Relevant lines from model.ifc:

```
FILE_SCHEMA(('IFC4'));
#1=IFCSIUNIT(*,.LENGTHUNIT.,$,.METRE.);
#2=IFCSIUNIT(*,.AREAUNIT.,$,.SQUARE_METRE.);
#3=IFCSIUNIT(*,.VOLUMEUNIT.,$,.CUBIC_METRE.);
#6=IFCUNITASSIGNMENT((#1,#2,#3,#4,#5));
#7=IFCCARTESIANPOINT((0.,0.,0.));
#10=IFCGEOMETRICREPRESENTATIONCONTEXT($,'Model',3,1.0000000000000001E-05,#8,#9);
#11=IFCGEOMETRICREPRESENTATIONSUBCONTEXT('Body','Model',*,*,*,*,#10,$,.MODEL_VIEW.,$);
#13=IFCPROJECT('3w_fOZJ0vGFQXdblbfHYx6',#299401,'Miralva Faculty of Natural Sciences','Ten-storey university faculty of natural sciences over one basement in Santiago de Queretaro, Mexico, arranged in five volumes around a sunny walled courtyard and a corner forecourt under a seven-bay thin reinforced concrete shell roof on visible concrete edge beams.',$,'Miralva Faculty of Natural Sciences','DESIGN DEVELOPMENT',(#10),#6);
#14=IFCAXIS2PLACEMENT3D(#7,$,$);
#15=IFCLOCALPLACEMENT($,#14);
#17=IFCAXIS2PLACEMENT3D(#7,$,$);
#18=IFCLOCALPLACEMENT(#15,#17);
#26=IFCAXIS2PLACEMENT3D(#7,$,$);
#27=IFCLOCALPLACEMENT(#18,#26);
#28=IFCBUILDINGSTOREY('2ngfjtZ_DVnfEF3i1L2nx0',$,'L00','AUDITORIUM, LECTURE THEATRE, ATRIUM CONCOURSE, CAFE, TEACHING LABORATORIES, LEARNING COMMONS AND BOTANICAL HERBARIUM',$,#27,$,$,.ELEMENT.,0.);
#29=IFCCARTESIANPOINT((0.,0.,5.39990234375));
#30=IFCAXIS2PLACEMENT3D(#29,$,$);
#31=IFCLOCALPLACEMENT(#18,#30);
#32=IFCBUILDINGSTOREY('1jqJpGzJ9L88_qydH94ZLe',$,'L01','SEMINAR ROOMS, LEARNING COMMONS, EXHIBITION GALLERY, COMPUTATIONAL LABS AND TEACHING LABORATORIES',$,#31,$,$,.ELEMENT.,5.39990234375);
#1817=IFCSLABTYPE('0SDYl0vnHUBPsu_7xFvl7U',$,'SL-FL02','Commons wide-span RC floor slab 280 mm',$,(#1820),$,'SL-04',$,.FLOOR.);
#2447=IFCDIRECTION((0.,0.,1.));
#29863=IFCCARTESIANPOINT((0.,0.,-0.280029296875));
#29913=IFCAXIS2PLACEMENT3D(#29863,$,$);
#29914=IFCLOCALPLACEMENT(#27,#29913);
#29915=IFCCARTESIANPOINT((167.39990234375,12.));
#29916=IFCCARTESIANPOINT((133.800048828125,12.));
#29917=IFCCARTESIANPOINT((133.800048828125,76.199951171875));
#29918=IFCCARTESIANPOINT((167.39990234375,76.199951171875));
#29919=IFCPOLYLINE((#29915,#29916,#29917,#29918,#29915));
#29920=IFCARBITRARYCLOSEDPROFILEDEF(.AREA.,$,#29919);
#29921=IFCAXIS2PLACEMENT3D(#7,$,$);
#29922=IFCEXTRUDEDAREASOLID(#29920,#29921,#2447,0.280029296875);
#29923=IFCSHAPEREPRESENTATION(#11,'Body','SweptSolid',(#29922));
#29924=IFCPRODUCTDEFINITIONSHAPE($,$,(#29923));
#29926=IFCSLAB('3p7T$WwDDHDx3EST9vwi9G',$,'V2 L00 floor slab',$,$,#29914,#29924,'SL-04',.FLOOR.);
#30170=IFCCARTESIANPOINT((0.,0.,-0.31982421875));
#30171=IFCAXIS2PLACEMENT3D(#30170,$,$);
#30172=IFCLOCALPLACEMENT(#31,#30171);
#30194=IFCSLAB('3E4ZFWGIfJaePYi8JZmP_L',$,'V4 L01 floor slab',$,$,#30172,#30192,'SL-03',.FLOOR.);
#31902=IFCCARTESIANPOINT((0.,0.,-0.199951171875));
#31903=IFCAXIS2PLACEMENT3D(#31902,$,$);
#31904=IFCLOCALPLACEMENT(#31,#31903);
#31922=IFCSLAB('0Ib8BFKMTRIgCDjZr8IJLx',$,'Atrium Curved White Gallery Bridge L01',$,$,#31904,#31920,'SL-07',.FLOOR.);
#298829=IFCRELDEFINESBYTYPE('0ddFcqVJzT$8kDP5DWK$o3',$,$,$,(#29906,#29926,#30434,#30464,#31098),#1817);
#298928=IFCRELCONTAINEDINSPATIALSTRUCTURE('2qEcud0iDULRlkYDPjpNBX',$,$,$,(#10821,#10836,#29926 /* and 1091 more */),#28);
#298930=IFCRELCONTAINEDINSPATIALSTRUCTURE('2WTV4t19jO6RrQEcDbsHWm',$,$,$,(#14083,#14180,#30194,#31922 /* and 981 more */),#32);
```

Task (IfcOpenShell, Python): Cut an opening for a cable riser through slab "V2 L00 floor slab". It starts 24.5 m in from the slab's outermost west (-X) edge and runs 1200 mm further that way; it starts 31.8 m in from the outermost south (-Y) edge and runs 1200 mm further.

```python
import numpy as np
import ifcopenshell
import ifcopenshell.api.feature
import ifcopenshell.api.geometry
import ifcopenshell.api.root
import ifcopenshell.geom
import ifcopenshell.util.placement
import ifcopenshell.util.representation
import ifcopenshell.util.shape
import ifcopenshell.util.unit

model = ifcopenshell.open("model.ifc")
unit_scale = ifcopenshell.util.unit.calculate_unit_scale(model)
settings = ifcopenshell.geom.settings()


def volume(element):
    """Net volume in cubic metres, openings subtracted."""
    shape = ifcopenshell.geom.create_shape(settings, element)
    return ifcopenshell.util.shape.get_volume(shape.geometry)


slab = model.by_guid("3p7T$WwDDHDx3EST9vwi9G")
before = volume(slab)

# Extent in the slab's own axes, in metres. The edges named are its -X and -Y sides.
slab_shape = ifcopenshell.geom.create_shape(settings, slab)
vertices = ifcopenshell.util.shape.get_vertices(slab_shape.geometry)
x_min, y_min, bottom = vertices.min(axis=0)
top = vertices[:, 2].max()

opening = ifcopenshell.api.root.create_entity(model, ifc_class="IfcOpeningElement", name="Cable riser opening", predefined_type="OPENING")
context = ifcopenshell.util.representation.get_context(model, "Model", "Body", "MODEL_VIEW")
width, depth = 1.2, 1.2
outline = [(0.0, 0.0), (width, 0.0), (width, depth), (0.0, depth), (0.0, 0.0)]
# Overshoot both faces by 50 mm so the cut is clean.
shape = ifcopenshell.api.geometry.add_slab_representation(
    model, context=context, depth=top - bottom + 0.1, polyline=outline
)
ifcopenshell.api.geometry.assign_representation(model, product=opening, representation=shape)

matrix = ifcopenshell.util.placement.get_local_placement(slab.ObjectPlacement)
matrix[:, 3] = matrix @ np.append(np.array([x_min + 24.5, y_min + 31.8, bottom - 0.05]) / unit_scale, 1.0)
ifcopenshell.api.geometry.edit_object_placement(model, product=opening, matrix=matrix, is_si=False)
ifcopenshell.api.feature.add_feature(model, feature=opening, element=slab)

after = volume(slab)

print(f"slab volume {before:.3f} -> {after:.3f} m3")

model.write("model_v2.ifc")
```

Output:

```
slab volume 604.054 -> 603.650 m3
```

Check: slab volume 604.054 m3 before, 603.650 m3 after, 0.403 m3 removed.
